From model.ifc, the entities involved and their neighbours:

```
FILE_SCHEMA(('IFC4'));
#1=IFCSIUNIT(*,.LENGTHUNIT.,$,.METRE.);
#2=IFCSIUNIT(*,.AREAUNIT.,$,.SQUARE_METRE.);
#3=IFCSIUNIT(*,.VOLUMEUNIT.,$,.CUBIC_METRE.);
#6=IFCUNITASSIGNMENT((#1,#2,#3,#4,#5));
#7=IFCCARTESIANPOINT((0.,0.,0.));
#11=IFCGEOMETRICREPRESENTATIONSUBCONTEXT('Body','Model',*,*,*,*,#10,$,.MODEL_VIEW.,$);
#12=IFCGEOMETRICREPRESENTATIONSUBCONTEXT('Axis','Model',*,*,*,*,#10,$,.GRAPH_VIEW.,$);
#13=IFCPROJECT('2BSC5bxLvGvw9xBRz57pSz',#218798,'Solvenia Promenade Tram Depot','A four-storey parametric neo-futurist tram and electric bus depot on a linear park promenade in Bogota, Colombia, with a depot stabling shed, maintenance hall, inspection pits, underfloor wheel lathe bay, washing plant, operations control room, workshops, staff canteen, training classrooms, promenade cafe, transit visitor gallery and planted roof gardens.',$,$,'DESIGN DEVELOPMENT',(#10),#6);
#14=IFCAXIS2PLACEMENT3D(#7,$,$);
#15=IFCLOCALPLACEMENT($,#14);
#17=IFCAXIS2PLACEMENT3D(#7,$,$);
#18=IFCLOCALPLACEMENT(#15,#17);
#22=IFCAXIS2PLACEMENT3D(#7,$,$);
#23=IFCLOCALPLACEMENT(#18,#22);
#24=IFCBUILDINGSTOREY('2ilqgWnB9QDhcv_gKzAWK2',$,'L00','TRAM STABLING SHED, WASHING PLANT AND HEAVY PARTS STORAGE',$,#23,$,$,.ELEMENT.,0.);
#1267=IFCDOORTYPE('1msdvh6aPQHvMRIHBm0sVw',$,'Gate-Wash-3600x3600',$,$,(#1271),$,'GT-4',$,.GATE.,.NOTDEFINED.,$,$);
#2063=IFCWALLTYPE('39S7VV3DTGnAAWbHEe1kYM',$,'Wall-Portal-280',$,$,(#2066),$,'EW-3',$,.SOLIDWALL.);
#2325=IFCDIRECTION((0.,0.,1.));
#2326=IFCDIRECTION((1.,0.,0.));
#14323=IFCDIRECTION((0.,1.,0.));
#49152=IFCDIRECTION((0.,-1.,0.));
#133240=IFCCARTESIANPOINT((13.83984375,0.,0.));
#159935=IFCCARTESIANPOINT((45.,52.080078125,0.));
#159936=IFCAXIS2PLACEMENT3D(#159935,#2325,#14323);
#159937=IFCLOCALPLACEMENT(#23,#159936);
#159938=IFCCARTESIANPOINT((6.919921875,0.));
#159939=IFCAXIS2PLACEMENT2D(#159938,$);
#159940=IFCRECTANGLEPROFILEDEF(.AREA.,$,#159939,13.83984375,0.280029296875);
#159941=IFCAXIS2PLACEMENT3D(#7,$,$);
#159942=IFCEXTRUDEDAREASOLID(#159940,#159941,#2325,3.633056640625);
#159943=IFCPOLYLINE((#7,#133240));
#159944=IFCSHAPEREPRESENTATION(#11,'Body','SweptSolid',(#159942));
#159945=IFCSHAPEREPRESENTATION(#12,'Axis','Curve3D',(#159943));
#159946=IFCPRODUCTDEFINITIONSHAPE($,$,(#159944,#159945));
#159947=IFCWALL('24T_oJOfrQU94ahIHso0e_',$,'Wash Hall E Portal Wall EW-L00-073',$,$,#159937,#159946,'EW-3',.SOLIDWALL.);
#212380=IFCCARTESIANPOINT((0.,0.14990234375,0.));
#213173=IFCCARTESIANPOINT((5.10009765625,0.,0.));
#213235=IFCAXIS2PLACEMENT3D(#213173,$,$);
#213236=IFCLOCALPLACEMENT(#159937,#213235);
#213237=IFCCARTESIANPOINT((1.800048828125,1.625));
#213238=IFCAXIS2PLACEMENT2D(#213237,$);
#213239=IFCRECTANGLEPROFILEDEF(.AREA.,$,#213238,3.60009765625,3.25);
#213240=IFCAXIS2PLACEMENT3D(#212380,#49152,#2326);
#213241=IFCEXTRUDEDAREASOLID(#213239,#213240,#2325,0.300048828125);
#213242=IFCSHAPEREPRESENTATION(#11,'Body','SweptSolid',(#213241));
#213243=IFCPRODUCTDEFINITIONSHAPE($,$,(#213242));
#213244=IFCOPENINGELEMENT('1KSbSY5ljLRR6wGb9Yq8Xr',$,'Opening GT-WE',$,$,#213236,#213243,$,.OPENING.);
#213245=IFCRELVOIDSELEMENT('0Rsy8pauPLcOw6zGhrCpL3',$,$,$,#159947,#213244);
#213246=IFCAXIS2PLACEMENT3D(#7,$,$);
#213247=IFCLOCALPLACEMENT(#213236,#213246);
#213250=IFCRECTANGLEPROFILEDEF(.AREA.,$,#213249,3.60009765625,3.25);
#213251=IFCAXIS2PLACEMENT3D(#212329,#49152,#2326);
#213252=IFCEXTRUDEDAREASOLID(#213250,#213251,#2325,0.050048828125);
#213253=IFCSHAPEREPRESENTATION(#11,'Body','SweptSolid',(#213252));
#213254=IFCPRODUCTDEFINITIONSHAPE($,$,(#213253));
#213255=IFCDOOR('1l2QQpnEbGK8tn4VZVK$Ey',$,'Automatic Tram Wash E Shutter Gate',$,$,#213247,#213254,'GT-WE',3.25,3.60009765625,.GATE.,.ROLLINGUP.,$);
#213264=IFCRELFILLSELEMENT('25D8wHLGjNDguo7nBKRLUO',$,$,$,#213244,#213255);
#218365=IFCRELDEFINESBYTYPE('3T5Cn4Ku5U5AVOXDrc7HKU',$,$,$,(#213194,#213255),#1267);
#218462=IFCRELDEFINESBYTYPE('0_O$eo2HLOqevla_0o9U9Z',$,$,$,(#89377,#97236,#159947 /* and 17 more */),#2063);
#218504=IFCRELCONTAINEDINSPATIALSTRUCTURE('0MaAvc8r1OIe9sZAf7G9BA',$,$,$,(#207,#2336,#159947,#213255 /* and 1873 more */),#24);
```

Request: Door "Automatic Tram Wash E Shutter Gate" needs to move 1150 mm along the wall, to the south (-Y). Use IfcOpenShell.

```python
import ifcopenshell
import ifcopenshell.api.geometry
import ifcopenshell.util.placement
import ifcopenshell.util.unit

model = ifcopenshell.open("model.ifc")
unit_scale = ifcopenshell.util.unit.calculate_unit_scale(model)

door = model.by_id(213255)
opening = door.FillsVoids[0].RelatingOpeningElement
wall = opening.VoidsElements[0].RelatingBuildingElement

wall_matrix = ifcopenshell.util.placement.get_local_placement(wall.ObjectPlacement)
shift = wall_matrix[:3, 0] * -1.15 / unit_scale
before = ifcopenshell.util.placement.get_local_placement(door.ObjectPlacement)[:3, 3].copy()

# The door is placed relative to its opening, so it follows when the opening moves.
matrix = ifcopenshell.util.placement.get_local_placement(opening.ObjectPlacement)
matrix[:3, 3] += shift
ifcopenshell.api.geometry.edit_object_placement(
    model, product=opening, matrix=matrix, is_si=False, should_transform_children=True
)

after = ifcopenshell.util.placement.get_local_placement(door.ObjectPlacement)[:3, 3]
print("door moved by", (after - before).round(3) + 0.0)

model.write("model-out.ifc")
```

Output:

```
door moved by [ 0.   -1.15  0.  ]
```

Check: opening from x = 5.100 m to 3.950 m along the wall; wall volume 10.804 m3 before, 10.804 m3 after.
